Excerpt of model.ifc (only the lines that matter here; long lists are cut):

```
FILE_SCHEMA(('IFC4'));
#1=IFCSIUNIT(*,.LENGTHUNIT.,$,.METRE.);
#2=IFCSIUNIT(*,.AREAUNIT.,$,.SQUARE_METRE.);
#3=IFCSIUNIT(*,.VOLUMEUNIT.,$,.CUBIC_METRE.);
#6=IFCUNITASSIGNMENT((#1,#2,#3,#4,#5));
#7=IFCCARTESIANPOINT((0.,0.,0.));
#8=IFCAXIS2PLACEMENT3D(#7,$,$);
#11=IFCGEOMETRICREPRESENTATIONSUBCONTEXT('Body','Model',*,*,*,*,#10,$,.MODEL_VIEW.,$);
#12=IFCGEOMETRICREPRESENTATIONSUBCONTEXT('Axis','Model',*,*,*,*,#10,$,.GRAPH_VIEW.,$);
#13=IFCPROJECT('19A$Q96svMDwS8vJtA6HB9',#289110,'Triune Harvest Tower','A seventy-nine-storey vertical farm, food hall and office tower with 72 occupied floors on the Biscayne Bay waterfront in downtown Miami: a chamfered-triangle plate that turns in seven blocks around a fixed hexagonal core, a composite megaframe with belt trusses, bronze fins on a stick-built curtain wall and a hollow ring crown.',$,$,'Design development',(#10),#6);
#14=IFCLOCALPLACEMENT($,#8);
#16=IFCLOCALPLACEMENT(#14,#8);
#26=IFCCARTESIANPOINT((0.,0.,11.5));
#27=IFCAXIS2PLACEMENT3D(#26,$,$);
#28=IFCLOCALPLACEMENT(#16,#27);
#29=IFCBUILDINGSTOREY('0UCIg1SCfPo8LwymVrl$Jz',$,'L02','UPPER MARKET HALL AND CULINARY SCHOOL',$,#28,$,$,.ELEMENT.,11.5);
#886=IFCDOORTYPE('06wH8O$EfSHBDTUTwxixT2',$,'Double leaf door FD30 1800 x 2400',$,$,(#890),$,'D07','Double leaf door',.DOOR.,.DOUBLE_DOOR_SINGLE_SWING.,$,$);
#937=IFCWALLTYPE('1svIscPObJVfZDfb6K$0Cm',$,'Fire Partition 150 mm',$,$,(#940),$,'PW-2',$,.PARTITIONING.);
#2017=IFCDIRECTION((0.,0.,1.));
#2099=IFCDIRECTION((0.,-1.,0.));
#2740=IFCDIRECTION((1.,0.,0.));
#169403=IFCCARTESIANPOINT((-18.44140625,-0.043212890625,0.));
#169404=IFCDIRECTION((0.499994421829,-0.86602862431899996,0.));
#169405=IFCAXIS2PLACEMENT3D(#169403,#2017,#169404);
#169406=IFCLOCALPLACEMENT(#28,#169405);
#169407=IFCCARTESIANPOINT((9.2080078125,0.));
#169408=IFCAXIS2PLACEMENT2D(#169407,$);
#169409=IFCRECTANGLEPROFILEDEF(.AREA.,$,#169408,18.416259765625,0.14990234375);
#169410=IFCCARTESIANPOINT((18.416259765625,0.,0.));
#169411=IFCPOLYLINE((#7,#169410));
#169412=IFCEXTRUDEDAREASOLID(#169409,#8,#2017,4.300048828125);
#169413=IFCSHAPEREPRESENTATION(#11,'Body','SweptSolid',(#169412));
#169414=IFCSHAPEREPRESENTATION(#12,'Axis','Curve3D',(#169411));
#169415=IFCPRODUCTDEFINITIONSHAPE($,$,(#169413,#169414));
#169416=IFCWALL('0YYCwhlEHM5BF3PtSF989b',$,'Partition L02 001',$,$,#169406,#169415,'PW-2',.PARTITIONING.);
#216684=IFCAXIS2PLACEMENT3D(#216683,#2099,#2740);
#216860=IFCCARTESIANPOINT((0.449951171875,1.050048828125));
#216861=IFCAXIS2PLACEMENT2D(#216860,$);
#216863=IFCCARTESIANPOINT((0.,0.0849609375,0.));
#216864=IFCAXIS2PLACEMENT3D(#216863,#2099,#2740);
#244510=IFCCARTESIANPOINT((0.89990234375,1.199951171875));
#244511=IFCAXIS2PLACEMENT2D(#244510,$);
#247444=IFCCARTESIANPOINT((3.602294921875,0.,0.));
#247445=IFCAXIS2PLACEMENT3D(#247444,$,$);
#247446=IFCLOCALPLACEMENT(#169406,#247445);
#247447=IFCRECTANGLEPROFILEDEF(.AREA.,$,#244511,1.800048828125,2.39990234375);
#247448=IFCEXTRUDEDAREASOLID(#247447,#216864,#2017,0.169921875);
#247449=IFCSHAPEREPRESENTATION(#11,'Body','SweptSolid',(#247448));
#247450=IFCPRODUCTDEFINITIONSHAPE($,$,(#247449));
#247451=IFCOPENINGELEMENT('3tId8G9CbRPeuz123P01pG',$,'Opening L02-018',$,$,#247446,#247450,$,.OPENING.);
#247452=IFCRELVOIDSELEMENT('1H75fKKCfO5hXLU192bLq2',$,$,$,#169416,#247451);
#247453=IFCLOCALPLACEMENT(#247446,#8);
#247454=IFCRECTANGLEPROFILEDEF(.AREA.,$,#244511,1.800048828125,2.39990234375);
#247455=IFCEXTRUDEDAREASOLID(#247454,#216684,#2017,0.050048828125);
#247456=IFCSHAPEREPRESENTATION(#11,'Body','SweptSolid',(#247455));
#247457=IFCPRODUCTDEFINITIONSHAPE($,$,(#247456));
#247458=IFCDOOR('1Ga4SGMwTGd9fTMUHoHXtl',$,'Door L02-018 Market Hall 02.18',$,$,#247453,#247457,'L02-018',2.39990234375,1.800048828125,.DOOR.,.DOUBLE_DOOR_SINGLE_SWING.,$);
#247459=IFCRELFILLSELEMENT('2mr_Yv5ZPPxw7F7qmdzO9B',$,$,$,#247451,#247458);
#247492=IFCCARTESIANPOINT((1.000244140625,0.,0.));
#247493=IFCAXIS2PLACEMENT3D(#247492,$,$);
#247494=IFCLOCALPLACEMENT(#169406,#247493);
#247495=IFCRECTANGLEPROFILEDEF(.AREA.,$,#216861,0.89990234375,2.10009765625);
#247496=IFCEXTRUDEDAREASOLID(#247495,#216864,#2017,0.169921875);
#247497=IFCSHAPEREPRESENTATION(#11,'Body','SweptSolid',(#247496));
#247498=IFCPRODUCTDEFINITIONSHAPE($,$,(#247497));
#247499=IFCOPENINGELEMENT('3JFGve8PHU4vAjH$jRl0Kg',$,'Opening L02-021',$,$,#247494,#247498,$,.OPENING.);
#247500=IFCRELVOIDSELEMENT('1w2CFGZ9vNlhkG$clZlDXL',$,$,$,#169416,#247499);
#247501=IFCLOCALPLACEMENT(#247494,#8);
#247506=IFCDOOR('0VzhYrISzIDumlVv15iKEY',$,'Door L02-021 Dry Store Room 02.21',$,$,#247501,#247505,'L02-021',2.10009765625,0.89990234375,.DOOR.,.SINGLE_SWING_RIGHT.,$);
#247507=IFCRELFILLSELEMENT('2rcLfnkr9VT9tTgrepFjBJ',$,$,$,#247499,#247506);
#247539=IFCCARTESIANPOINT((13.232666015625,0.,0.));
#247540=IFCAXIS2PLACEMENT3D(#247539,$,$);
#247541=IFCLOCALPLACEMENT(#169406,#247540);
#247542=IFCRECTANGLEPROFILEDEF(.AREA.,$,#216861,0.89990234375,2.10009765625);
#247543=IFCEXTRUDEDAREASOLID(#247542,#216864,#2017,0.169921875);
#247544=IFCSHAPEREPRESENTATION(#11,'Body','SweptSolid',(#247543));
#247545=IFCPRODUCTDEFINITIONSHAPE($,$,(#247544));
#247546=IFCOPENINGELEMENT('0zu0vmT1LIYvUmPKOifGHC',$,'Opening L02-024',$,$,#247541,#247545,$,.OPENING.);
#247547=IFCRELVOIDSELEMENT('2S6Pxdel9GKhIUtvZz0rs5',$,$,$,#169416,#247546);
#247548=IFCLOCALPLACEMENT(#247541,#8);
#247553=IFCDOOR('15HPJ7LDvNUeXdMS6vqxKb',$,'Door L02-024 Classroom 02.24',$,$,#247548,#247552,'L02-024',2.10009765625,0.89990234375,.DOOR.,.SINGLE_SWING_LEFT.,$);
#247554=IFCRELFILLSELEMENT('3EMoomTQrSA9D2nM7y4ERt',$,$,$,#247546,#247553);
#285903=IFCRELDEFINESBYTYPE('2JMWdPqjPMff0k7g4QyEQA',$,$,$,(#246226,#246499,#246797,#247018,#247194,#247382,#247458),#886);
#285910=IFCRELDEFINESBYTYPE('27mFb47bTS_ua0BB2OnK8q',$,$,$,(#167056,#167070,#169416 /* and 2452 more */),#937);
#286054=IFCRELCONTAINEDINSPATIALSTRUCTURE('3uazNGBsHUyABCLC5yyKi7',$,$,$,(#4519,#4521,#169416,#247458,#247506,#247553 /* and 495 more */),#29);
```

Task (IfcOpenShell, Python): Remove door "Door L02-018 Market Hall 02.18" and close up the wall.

```python
import ifcopenshell
import ifcopenshell.api.feature
import ifcopenshell.api.root
import ifcopenshell.geom
import ifcopenshell.util.shape

model = ifcopenshell.open("model.ifc")
settings = ifcopenshell.geom.settings()


def volume(element):
    """Net volume in cubic metres, openings subtracted."""
    shape = ifcopenshell.geom.create_shape(settings, element)
    return ifcopenshell.util.shape.get_volume(shape.geometry)


door = model.by_guid("1Ga4SGMwTGd9fTMUHoHXtl")
opening = door.FillsVoids[0].RelatingOpeningElement
wall = opening.VoidsElements[0].RelatingBuildingElement
before = volume(wall)

ifcopenshell.api.root.remove_product(model, product=door)
ifcopenshell.api.feature.remove_feature(model, feature=opening)

after = volume(wall)

print(f"wall volume {before:.3f} -> {after:.3f} m3")

model.write("model_edited.ifc")
```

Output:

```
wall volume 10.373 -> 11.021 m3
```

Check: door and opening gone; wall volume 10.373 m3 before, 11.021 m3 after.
